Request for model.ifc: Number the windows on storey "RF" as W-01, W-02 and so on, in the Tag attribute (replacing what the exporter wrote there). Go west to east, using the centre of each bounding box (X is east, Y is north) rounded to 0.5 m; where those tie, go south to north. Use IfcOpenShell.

First a look at what the model holds.

```python
import ifcopenshell
import ifcopenshell.util.element
import ifcopenshell.util.placement

model = ifcopenshell.open("model.ifc")
print(model.schema)
storey = next(s for s in model.by_type("IfcBuildingStorey") if s.Name == "RF")
windows = [e for e in ifcopenshell.util.element.get_decomposition(storey) if e.is_a("IfcWindow")]
for e in sorted(windows, key=lambda e: e.id()):
    origin = ifcopenshell.util.placement.get_local_placement(e.ObjectPlacement)[:3, 3]
    print(e.id(), e.Tag, e.Name, origin.round(2) + 0.0, sep=" | ")
```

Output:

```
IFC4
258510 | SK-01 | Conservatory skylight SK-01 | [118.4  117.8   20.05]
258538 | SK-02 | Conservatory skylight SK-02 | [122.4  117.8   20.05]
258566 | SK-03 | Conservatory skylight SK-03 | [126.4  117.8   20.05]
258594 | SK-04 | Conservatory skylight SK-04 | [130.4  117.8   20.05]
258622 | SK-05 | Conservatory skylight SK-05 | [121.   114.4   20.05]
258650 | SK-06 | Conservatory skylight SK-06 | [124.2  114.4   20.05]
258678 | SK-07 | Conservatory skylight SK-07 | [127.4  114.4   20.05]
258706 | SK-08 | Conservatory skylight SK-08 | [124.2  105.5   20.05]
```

```python
import ifcopenshell
import ifcopenshell.geom
import ifcopenshell.util.element
import ifcopenshell.util.shape

model = ifcopenshell.open("model.ifc")
settings = ifcopenshell.geom.settings()
settings.set("use-world-coords", True)


def centre(element):
    shape = ifcopenshell.geom.create_shape(settings, element)
    return ifcopenshell.util.shape.get_bbox_centroid(shape.geometry)


storey = next(s for s in model.by_type("IfcBuildingStorey") if s.Name == "RF")
windows = [e for e in ifcopenshell.util.element.get_decomposition(storey) if e.is_a("IfcWindow")]

# Insertion points can sit at a corner or the storey origin, so sort by the geometry (in metres).
centres = {e: centre(e) for e in windows}
windows.sort(key=lambda e: (round(centres[e][0] / 0.5), centres[e][1]))

for i, e in enumerate(windows, start=1):
    number = f"W-{i:02d}"
    e.Tag = number
    print(e.id(), number)

model.write("model_edited.ifc")
```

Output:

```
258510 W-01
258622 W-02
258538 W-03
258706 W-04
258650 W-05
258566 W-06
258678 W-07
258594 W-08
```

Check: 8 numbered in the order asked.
